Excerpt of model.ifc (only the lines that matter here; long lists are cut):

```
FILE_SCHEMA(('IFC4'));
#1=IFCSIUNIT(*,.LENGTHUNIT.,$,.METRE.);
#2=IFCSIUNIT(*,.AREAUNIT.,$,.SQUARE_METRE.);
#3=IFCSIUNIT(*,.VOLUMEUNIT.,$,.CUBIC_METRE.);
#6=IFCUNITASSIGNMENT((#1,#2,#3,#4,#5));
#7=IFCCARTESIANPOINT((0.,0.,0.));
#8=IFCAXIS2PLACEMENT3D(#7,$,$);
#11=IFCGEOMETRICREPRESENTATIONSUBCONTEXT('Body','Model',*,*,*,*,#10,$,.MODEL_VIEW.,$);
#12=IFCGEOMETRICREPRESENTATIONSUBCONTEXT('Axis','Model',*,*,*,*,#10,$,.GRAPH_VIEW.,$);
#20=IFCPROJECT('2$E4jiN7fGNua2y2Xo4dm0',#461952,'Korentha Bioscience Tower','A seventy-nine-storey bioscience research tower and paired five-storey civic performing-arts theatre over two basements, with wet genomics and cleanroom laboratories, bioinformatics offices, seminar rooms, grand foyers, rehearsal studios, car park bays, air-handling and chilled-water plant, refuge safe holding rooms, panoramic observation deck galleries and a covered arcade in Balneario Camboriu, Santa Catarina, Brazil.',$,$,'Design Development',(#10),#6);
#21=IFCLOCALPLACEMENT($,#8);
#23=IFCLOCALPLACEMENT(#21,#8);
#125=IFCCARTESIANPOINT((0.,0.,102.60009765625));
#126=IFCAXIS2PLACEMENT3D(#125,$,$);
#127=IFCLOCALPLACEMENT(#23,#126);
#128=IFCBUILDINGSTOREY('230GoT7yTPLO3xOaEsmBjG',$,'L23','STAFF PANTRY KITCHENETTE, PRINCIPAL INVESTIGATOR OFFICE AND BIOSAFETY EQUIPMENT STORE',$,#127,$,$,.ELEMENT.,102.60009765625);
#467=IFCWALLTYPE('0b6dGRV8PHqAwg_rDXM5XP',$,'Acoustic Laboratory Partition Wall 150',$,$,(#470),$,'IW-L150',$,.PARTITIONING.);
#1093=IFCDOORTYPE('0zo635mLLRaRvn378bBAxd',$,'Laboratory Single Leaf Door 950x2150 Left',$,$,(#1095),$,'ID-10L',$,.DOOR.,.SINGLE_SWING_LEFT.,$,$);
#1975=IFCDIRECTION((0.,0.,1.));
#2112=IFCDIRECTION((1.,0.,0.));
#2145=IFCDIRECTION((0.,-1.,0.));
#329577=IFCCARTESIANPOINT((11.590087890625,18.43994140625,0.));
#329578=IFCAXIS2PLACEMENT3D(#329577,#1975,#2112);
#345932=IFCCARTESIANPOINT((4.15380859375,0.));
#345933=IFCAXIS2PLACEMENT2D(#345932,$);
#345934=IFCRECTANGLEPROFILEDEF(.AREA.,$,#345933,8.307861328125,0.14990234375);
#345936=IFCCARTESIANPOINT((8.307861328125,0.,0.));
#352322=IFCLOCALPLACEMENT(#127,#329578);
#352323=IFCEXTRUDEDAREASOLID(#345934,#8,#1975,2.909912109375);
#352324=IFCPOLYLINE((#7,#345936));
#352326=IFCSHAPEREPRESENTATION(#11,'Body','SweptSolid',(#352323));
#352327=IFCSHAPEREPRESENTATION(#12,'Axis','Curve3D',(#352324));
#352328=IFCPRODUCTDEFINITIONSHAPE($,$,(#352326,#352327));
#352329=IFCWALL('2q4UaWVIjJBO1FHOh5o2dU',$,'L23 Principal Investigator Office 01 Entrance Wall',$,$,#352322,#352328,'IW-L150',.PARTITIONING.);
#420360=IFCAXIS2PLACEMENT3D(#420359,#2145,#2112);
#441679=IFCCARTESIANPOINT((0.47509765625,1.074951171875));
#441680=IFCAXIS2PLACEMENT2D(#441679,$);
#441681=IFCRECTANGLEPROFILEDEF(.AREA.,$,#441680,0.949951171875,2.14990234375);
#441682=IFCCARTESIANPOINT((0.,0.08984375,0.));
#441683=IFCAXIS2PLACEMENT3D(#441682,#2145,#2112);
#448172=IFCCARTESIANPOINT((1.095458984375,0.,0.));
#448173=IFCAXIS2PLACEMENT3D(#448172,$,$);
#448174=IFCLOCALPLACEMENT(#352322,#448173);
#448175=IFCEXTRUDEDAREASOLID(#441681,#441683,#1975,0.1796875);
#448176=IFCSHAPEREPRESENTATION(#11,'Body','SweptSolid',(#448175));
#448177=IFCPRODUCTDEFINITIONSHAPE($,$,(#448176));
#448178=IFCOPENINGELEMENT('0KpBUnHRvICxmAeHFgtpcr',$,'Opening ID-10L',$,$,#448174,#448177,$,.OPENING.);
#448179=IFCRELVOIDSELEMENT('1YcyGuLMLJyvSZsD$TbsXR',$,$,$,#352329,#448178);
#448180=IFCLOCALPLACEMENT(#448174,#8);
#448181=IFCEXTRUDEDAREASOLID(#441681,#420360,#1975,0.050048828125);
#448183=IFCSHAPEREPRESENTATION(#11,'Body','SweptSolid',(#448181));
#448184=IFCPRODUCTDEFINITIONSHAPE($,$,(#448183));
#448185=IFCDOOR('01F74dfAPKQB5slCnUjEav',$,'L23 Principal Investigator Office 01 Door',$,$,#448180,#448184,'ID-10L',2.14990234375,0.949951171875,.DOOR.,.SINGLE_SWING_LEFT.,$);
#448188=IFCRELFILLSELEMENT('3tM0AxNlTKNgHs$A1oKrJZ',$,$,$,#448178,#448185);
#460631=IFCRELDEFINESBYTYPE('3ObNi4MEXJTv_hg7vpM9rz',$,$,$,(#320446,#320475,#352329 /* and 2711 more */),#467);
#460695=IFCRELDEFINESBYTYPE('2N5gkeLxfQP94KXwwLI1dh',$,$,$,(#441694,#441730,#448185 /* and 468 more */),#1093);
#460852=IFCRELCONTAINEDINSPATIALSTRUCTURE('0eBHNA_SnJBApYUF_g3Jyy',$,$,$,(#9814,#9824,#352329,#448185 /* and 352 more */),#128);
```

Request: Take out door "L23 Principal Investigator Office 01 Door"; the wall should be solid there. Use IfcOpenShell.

```python
import ifcopenshell
import ifcopenshell.api.feature
import ifcopenshell.api.root
import ifcopenshell.geom
import ifcopenshell.util.shape

model = ifcopenshell.open("model.ifc")
settings = ifcopenshell.geom.settings()


def volume(element):
    """Net volume in cubic metres, openings subtracted."""
    shape = ifcopenshell.geom.create_shape(settings, element)
    return ifcopenshell.util.shape.get_volume(shape.geometry)


door = model.by_guid("01F74dfAPKQB5slCnUjEav")
opening = door.FillsVoids[0].RelatingOpeningElement
wall = opening.VoidsElements[0].RelatingBuildingElement
before = volume(wall)

ifcopenshell.api.root.remove_product(model, product=door)
ifcopenshell.api.feature.remove_feature(model, feature=opening)

after = volume(wall)

print(f"wall volume {before:.3f} -> {after:.3f} m3")

model.write("model_updated.ifc")
```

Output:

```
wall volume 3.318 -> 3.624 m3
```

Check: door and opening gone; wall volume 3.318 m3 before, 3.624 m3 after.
